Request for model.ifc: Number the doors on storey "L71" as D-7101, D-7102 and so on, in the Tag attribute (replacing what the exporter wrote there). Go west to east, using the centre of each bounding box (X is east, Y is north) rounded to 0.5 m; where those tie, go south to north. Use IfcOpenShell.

First a look at what the model holds.

```python
import ifcopenshell
import ifcopenshell.util.element
import ifcopenshell.util.placement

model = ifcopenshell.open("model.ifc")
print(model.schema)
storey = next(s for s in model.by_type("IfcBuildingStorey") if s.Name == "L71")
doors = [e for e in ifcopenshell.util.element.get_decomposition(storey) if e.is_a("IfcDoor")]
for e in sorted(doors, key=lambda e: e.id()):
    origin = ifcopenshell.util.placement.get_local_placement(e.ObjectPlacement)[:3, 3]
    print(e.id(), e.Tag, e.Name, origin.round(2) + 0.0, sep=" | ")
```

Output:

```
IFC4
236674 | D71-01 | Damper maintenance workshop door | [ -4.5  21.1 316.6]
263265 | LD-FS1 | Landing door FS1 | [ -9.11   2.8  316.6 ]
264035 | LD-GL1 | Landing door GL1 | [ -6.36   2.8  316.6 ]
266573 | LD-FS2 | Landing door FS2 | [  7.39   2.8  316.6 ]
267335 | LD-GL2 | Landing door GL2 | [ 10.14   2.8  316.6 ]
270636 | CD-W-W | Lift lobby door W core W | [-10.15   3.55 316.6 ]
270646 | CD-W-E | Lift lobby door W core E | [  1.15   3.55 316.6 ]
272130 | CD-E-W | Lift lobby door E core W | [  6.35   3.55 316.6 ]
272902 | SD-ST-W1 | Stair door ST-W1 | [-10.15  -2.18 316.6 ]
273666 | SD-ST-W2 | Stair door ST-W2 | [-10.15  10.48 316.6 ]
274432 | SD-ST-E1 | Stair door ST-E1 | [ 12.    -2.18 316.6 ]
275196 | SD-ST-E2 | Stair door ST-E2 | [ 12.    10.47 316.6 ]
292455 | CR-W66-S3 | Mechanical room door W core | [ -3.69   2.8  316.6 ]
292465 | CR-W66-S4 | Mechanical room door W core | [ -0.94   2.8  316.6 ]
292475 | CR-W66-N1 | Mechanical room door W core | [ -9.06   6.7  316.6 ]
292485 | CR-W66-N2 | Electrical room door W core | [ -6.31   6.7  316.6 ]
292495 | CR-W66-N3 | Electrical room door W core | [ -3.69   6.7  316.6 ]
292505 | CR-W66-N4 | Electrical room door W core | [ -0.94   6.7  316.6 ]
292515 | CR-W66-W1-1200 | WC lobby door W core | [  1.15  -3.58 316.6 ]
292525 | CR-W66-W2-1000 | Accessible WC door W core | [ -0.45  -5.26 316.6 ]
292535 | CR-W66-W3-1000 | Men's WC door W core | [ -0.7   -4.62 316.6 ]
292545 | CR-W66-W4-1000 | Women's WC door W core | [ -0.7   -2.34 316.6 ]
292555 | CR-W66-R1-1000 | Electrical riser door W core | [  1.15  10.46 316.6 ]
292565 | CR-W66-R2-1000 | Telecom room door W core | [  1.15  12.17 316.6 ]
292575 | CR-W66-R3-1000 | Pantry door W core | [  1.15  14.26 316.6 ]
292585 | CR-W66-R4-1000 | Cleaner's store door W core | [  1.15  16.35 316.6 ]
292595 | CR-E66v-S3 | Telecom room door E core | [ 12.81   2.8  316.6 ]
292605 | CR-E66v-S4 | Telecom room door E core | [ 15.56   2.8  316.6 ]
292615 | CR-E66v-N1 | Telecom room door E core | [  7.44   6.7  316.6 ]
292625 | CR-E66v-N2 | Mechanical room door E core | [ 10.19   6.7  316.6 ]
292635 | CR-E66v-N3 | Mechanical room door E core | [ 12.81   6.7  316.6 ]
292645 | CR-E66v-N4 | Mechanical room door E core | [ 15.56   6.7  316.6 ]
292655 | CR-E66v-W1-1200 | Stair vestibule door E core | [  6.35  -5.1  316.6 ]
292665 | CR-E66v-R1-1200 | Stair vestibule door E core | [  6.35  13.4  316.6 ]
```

```python
import ifcopenshell
import ifcopenshell.geom
import ifcopenshell.util.element
import ifcopenshell.util.shape

model = ifcopenshell.open("model.ifc")
settings = ifcopenshell.geom.settings()
settings.set("use-world-coords", True)


def centre(element):
    shape = ifcopenshell.geom.create_shape(settings, element)
    return ifcopenshell.util.shape.get_bbox_centroid(shape.geometry)


storey = next(s for s in model.by_type("IfcBuildingStorey") if s.Name == "L71")
doors = [e for e in ifcopenshell.util.element.get_decomposition(storey) if e.is_a("IfcDoor")]

# Insertion points can sit at a corner or the storey origin, so sort by the geometry (in metres).
centres = {e: centre(e) for e in doors}
doors.sort(key=lambda e: (round(centres[e][0] / 0.5), centres[e][1]))

for i, e in enumerate(doors, start=1):
    number = f"D-71{i:02d}"
    e.Tag = number
    print(e.id(), number)

model.write("model_updated.ifc")
```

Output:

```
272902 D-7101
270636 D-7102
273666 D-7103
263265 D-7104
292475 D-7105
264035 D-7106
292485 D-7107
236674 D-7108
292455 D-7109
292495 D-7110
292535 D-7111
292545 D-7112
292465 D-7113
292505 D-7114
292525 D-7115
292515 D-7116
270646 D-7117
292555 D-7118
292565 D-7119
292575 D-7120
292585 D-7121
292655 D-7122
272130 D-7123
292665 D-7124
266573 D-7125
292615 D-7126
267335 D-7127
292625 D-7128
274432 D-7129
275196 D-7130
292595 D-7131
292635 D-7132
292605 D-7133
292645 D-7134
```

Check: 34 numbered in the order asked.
